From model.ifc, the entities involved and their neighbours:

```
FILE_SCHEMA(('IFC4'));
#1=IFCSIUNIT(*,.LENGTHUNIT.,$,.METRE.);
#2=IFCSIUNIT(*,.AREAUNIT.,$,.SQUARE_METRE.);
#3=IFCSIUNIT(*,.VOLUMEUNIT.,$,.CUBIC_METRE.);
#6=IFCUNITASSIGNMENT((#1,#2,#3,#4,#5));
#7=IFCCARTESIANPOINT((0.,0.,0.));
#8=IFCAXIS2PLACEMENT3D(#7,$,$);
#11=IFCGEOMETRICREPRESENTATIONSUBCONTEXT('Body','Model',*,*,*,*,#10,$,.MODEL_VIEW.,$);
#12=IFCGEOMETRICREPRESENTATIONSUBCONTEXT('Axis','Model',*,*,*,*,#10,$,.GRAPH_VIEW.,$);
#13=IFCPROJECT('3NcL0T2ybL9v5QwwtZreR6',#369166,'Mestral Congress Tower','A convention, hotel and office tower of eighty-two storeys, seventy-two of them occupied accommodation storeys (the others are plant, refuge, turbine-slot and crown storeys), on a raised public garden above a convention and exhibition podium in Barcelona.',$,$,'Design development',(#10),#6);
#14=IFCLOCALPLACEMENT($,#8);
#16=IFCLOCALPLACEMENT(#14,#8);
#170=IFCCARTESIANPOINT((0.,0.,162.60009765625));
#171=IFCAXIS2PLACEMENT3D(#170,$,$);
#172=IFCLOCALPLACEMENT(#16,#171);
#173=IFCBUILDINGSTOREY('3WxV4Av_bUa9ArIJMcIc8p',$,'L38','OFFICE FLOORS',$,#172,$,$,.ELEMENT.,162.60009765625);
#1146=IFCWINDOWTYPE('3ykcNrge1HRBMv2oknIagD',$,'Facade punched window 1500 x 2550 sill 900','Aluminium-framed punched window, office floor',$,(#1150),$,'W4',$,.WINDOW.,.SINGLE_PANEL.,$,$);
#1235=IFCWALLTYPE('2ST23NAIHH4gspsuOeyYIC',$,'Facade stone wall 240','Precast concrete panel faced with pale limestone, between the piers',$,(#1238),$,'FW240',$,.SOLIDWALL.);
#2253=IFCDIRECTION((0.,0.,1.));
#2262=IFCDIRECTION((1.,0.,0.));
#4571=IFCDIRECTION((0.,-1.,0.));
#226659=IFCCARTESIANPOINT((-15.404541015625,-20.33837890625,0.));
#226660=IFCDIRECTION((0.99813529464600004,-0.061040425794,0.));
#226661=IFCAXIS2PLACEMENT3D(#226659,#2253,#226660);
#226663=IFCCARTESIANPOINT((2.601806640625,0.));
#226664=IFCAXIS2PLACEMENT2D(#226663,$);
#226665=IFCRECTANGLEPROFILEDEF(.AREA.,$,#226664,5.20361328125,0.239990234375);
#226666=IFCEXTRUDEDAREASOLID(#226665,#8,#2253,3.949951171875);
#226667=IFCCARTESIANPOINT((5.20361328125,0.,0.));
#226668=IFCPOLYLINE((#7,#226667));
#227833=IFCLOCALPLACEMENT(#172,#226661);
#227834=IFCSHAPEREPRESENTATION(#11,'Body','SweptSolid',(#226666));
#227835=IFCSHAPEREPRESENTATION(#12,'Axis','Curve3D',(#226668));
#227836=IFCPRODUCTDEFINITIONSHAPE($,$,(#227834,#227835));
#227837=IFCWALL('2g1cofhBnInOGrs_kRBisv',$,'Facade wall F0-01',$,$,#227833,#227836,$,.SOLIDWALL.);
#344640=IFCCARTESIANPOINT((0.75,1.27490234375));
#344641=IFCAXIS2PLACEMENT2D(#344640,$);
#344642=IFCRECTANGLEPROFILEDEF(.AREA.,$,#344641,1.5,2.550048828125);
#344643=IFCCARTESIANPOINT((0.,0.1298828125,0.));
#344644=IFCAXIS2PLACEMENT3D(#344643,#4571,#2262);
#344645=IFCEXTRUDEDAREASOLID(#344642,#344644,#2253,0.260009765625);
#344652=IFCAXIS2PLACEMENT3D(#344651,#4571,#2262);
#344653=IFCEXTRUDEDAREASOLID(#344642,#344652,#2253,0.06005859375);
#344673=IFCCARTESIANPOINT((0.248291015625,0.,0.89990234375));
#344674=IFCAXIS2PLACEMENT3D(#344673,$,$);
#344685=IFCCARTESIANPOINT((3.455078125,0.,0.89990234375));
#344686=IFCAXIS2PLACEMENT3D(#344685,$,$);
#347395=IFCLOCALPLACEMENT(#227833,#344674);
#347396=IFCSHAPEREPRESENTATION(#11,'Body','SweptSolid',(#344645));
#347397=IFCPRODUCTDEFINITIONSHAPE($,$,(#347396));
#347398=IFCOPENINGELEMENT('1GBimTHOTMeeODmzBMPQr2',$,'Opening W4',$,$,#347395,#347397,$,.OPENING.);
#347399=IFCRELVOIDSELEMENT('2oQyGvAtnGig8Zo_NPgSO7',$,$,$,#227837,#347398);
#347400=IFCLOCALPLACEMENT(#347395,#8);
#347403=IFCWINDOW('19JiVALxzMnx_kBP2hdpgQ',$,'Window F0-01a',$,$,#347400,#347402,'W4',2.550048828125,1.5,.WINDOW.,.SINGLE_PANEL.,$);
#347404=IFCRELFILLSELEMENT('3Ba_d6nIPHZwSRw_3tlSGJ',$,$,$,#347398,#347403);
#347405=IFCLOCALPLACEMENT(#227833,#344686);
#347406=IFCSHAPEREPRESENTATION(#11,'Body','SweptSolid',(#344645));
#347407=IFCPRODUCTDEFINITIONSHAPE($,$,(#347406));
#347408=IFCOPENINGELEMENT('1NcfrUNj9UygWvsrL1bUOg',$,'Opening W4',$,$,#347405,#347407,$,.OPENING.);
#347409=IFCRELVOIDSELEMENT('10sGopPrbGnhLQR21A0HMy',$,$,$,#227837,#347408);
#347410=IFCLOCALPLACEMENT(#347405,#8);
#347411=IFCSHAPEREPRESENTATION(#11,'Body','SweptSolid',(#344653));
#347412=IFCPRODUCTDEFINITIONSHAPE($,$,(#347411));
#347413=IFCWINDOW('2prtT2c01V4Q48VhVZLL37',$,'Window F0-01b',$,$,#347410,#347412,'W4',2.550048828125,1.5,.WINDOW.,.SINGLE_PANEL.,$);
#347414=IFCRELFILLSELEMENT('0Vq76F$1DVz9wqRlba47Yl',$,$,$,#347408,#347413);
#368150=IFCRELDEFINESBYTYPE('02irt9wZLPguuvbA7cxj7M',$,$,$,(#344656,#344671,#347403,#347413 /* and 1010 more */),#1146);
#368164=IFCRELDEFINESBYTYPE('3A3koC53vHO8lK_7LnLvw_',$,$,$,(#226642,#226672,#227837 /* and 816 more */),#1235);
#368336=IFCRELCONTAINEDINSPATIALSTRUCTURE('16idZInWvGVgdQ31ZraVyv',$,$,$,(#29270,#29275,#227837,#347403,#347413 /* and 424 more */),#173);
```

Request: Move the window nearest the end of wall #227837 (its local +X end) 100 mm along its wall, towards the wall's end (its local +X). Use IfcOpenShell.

```python
import ifcopenshell
import ifcopenshell.api.geometry
import ifcopenshell.util.placement

model = ifcopenshell.open("model.ifc")

window = model.by_guid("2prtT2c01V4Q48VhVZLL37")
opening = window.FillsVoids[0].RelatingOpeningElement
wall = opening.VoidsElements[0].RelatingBuildingElement

wall_matrix = ifcopenshell.util.placement.get_local_placement(wall.ObjectPlacement)
shift = wall_matrix[:3, 0] * 0.1
before = ifcopenshell.util.placement.get_local_placement(window.ObjectPlacement)[:3, 3].copy()

# The window is placed relative to its opening, so it follows when the opening moves.
matrix = ifcopenshell.util.placement.get_local_placement(opening.ObjectPlacement)
matrix[:3, 3] += shift
ifcopenshell.api.geometry.edit_object_placement(
    model, product=opening, matrix=matrix, is_si=False, should_transform_children=True
)

after = ifcopenshell.util.placement.get_local_placement(window.ObjectPlacement)[:3, 3]
print("window moved by", (after - before).round(3) + 0.0)

model.write("model-out.ifc")
```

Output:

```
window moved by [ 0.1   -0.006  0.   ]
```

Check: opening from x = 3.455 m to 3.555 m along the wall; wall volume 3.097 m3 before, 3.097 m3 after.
